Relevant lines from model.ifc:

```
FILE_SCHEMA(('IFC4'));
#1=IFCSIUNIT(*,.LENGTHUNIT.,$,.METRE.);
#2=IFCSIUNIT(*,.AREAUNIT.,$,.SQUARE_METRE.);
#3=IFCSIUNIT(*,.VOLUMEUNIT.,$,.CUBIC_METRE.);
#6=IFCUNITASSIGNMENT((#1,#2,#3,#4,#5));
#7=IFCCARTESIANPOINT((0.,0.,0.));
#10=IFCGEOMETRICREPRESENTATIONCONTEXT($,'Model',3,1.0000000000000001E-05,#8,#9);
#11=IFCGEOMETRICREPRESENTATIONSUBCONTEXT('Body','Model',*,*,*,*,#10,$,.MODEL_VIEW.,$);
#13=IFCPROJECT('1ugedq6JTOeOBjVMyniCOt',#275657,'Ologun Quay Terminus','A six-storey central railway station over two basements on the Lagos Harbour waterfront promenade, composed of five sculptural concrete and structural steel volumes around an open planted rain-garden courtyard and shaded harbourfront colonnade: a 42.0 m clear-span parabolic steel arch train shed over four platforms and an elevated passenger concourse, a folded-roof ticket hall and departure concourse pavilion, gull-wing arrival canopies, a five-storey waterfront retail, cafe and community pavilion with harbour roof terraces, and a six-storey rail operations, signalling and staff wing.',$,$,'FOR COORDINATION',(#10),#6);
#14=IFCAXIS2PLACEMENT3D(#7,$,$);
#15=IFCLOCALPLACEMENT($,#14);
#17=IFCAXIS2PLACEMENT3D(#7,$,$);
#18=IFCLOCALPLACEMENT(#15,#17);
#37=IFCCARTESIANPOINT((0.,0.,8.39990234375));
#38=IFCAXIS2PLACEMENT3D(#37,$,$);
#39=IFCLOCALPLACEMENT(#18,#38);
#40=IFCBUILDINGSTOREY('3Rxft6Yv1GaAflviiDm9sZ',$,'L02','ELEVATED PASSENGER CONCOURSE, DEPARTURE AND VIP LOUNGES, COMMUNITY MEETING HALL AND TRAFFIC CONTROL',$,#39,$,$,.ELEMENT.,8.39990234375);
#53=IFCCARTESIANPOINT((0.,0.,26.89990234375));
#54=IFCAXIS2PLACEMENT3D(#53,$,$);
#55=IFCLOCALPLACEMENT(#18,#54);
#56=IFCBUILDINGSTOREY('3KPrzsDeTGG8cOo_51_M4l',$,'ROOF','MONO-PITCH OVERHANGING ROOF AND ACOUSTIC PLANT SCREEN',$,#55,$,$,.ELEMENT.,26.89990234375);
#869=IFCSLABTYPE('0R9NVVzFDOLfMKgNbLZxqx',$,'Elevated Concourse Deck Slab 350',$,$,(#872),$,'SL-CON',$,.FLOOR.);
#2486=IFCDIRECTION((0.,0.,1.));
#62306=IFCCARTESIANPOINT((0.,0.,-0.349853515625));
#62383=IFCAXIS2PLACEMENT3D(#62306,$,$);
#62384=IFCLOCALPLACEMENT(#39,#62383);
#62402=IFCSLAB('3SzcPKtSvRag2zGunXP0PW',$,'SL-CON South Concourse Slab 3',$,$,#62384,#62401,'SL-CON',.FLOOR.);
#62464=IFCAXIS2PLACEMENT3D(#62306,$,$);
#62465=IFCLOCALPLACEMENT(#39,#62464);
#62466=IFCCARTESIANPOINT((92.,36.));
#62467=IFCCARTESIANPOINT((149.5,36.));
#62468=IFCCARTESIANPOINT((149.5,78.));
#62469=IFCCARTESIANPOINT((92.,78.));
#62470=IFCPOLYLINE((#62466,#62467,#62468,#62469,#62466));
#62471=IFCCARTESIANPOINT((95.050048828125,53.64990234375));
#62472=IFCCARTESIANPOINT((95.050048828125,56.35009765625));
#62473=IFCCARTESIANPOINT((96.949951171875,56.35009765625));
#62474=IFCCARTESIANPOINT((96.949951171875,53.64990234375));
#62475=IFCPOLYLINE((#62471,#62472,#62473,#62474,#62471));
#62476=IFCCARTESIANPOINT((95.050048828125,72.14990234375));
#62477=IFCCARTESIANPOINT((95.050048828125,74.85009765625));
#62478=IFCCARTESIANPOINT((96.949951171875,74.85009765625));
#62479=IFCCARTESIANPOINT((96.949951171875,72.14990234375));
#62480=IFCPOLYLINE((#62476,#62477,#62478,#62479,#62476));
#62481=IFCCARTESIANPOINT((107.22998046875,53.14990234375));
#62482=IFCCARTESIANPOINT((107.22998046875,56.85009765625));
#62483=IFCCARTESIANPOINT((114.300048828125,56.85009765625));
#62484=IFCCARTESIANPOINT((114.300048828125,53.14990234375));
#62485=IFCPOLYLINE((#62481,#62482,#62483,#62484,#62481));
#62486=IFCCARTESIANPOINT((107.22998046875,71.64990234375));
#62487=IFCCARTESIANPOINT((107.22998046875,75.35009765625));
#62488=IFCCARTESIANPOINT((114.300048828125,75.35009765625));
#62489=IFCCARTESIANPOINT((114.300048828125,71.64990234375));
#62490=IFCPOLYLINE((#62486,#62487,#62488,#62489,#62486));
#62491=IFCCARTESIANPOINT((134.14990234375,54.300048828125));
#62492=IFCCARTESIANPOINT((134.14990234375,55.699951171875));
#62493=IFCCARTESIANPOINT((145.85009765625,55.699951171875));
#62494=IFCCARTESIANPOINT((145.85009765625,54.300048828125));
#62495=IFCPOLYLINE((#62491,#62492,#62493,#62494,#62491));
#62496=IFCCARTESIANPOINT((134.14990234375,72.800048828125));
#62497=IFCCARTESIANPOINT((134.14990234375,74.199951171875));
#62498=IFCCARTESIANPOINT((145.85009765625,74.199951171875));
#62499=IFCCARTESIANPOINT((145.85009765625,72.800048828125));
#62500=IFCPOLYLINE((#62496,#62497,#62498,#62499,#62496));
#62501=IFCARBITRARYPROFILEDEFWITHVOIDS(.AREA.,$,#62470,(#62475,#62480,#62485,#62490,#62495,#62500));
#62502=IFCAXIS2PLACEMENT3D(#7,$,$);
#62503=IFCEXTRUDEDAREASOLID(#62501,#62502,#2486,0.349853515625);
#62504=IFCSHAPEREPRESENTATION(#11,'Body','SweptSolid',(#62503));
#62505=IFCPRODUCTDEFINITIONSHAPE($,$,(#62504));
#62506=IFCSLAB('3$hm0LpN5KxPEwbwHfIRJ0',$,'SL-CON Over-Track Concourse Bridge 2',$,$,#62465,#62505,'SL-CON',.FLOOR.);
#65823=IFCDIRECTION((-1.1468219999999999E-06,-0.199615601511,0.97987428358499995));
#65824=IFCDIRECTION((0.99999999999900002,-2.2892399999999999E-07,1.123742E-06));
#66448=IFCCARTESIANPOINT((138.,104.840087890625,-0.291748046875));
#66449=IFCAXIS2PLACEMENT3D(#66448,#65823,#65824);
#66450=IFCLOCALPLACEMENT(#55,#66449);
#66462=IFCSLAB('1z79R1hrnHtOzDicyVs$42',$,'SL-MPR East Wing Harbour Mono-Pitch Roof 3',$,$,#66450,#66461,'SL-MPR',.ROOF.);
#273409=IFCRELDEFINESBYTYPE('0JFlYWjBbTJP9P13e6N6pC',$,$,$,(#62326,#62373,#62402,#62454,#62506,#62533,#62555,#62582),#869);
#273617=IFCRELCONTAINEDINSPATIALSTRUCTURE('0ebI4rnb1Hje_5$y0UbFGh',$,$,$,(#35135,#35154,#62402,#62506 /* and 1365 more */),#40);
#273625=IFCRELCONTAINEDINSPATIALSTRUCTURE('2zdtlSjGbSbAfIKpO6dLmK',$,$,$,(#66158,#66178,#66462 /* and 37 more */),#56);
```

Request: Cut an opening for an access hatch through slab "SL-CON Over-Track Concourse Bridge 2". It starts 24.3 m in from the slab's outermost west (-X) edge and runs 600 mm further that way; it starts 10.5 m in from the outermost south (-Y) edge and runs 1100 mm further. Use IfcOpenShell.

```python
import numpy as np
import ifcopenshell
import ifcopenshell.api.feature
import ifcopenshell.api.geometry
import ifcopenshell.api.root
import ifcopenshell.geom
import ifcopenshell.util.placement
import ifcopenshell.util.representation
import ifcopenshell.util.shape
import ifcopenshell.util.unit

model = ifcopenshell.open("model.ifc")
unit_scale = ifcopenshell.util.unit.calculate_unit_scale(model)
settings = ifcopenshell.geom.settings()


def volume(element):
    """Net volume in cubic metres, openings subtracted."""
    shape = ifcopenshell.geom.create_shape(settings, element)
    return ifcopenshell.util.shape.get_volume(shape.geometry)


slab = model.by_guid("3$hm0LpN5KxPEwbwHfIRJ0")
before = volume(slab)

# Extent in the slab's own axes, in metres. The edges named are its -X and -Y sides.
slab_shape = ifcopenshell.geom.create_shape(settings, slab)
vertices = ifcopenshell.util.shape.get_vertices(slab_shape.geometry)
x_min, y_min, bottom = vertices.min(axis=0)
top = vertices[:, 2].max()

opening = ifcopenshell.api.root.create_entity(model, ifc_class="IfcOpeningElement", name="Access hatch opening", predefined_type="OPENING")
context = ifcopenshell.util.representation.get_context(model, "Model", "Body", "MODEL_VIEW")
width, depth = 0.6, 1.1
outline = [(0.0, 0.0), (width, 0.0), (width, depth), (0.0, depth), (0.0, 0.0)]
# Overshoot both faces by 50 mm so the cut is clean.
shape = ifcopenshell.api.geometry.add_slab_representation(
    model, context=context, depth=top - bottom + 0.1, polyline=outline
)
ifcopenshell.api.geometry.assign_representation(model, product=opening, representation=shape)

matrix = ifcopenshell.util.placement.get_local_placement(slab.ObjectPlacement)
matrix[:, 3] = matrix @ np.append(np.array([x_min + 24.3, y_min + 10.5, bottom - 0.05]) / unit_scale, 1.0)
ifcopenshell.api.geometry.edit_object_placement(model, product=opening, matrix=matrix, is_si=False)
ifcopenshell.api.feature.add_feature(model, feature=opening, element=slab)

after = volume(slab)

print(f"slab volume {before:.3f} -> {after:.3f} m3")

model.write("model-out.ifc")
```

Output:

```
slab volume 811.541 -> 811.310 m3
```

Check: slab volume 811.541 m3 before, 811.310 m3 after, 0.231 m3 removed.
